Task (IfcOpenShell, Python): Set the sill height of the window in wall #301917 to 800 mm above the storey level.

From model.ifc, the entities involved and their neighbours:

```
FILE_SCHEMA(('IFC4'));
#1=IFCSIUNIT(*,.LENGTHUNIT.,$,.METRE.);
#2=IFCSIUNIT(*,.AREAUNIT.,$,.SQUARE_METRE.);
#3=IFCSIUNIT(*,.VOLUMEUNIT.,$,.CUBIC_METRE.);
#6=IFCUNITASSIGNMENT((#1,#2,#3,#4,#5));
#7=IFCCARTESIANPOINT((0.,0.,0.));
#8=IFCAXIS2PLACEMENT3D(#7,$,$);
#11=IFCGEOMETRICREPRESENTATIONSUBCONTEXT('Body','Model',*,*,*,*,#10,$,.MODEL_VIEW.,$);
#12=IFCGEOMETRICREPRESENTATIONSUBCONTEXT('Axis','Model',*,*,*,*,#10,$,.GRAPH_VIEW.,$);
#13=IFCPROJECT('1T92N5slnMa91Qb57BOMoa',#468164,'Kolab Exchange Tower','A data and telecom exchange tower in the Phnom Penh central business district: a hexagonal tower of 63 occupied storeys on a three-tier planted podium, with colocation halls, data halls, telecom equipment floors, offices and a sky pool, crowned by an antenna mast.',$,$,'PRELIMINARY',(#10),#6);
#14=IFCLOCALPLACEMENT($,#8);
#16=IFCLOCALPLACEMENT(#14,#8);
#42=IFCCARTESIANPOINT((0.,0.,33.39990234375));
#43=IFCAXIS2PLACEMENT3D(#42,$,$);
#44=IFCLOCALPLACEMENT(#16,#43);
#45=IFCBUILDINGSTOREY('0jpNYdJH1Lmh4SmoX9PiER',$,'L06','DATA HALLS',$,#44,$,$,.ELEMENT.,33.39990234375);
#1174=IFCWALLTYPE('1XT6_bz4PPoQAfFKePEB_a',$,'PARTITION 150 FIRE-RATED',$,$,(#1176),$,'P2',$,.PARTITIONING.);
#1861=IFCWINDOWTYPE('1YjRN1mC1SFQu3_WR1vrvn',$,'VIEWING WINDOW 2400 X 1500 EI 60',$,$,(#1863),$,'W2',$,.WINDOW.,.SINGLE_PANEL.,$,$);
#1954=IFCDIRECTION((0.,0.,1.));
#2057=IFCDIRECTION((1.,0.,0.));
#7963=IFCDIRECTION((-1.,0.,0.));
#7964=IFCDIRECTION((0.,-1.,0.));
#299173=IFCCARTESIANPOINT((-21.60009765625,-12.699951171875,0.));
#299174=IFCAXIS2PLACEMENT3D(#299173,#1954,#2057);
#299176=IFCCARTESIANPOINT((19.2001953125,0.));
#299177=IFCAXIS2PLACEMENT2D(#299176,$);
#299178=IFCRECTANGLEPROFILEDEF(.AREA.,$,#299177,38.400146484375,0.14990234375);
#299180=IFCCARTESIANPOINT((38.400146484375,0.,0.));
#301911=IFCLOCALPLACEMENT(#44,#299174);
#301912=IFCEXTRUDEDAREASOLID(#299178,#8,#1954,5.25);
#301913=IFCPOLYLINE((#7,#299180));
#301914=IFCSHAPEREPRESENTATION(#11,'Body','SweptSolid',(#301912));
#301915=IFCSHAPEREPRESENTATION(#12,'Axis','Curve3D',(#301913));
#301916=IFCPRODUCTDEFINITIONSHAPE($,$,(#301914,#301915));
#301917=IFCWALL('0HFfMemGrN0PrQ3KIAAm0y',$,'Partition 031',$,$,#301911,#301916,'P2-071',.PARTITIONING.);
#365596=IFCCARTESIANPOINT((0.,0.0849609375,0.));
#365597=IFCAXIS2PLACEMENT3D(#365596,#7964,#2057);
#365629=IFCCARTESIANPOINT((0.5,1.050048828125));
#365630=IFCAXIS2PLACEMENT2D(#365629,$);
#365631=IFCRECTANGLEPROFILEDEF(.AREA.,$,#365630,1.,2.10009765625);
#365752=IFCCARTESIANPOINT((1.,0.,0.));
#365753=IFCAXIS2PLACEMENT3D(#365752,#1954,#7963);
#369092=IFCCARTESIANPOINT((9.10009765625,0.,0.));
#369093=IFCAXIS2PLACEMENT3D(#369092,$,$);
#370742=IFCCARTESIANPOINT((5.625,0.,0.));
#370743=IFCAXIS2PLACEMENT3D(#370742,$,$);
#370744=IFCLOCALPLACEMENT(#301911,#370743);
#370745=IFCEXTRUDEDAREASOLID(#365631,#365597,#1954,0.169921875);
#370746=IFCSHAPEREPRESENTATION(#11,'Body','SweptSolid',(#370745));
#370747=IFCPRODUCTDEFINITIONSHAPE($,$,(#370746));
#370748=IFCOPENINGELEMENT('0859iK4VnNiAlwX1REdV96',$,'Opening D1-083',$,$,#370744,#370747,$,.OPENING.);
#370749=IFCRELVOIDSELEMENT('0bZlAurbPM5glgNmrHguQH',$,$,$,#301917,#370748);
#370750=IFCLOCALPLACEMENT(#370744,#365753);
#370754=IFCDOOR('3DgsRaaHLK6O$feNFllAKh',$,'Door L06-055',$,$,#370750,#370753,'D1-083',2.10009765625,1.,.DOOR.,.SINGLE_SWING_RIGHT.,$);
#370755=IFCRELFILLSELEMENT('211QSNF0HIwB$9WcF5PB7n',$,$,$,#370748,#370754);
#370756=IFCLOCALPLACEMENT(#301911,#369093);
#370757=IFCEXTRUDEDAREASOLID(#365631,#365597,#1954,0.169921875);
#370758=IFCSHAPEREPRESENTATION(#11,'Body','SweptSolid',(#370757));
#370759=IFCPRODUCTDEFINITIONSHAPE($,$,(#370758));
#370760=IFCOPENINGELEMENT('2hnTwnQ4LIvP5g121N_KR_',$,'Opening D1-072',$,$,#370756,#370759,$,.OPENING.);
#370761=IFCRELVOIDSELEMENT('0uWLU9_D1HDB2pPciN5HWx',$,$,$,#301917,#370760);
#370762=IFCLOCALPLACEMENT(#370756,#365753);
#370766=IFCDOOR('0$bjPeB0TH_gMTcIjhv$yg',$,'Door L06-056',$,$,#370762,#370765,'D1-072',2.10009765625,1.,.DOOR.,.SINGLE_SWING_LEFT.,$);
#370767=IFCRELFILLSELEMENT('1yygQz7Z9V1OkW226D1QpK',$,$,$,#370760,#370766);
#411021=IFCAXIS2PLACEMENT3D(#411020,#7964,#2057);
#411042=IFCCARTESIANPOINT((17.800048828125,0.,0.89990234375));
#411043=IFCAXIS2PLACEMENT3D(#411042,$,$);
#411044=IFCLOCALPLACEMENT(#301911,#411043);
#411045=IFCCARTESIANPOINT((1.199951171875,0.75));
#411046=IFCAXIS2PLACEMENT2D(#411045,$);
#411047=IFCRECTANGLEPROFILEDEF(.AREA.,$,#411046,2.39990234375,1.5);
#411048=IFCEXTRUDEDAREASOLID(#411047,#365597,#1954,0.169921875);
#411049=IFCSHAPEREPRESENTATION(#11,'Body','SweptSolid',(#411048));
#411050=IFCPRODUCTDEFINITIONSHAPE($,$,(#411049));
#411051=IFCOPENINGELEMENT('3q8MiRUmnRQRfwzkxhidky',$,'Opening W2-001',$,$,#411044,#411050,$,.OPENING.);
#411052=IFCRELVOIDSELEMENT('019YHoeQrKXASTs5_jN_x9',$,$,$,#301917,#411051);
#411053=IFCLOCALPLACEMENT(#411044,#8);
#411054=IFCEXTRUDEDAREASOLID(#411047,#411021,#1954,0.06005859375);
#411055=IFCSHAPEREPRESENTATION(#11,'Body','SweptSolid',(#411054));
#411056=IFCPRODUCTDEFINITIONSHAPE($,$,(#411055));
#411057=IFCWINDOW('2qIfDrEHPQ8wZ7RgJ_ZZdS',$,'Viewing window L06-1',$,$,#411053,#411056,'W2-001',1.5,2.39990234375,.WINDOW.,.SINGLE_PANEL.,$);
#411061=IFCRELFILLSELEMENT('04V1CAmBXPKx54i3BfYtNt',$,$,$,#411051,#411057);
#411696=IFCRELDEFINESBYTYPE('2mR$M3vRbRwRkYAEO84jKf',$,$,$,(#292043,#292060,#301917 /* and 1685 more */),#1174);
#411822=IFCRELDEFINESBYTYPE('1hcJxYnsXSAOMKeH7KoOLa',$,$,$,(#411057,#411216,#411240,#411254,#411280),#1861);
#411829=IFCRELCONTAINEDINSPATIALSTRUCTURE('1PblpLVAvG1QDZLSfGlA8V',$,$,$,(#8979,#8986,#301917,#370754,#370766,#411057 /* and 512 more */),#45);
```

```python
import numpy as np
import ifcopenshell
import ifcopenshell.api.geometry
import ifcopenshell.geom
import ifcopenshell.util.element
import ifcopenshell.util.placement
import ifcopenshell.util.shape
import ifcopenshell.util.unit

model = ifcopenshell.open("model.ifc")
unit_scale = ifcopenshell.util.unit.calculate_unit_scale(model)

window = model.by_id(411057)
opening = window.FillsVoids[0].RelatingOpeningElement
storey = ifcopenshell.util.element.get_container(window, ifc_class="IfcBuildingStorey")
level = ifcopenshell.util.placement.get_local_placement(storey.ObjectPlacement)[2, 3]

# The opening's origin need not be at the sill, so measure its lowest point.
shape = ifcopenshell.geom.create_shape(ifcopenshell.geom.settings(), opening)
bottom = ifcopenshell.util.shape.get_shape_bottom_elevation(shape, shape.geometry) / unit_scale
dz = level + 0.8 / unit_scale - bottom

shift = np.array([0.0, 0.0, dz])
# The window is placed relative to its opening, so it follows when the opening moves.
matrix = ifcopenshell.util.placement.get_local_placement(opening.ObjectPlacement)
matrix[:3, 3] += shift
ifcopenshell.api.geometry.edit_object_placement(
    model, product=opening, matrix=matrix, is_si=False, should_transform_children=True
)

print(f"moved by {dz * unit_scale:+.3f} m")

model.write("model_v2.ifc")
```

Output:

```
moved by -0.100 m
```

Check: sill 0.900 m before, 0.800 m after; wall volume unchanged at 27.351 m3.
